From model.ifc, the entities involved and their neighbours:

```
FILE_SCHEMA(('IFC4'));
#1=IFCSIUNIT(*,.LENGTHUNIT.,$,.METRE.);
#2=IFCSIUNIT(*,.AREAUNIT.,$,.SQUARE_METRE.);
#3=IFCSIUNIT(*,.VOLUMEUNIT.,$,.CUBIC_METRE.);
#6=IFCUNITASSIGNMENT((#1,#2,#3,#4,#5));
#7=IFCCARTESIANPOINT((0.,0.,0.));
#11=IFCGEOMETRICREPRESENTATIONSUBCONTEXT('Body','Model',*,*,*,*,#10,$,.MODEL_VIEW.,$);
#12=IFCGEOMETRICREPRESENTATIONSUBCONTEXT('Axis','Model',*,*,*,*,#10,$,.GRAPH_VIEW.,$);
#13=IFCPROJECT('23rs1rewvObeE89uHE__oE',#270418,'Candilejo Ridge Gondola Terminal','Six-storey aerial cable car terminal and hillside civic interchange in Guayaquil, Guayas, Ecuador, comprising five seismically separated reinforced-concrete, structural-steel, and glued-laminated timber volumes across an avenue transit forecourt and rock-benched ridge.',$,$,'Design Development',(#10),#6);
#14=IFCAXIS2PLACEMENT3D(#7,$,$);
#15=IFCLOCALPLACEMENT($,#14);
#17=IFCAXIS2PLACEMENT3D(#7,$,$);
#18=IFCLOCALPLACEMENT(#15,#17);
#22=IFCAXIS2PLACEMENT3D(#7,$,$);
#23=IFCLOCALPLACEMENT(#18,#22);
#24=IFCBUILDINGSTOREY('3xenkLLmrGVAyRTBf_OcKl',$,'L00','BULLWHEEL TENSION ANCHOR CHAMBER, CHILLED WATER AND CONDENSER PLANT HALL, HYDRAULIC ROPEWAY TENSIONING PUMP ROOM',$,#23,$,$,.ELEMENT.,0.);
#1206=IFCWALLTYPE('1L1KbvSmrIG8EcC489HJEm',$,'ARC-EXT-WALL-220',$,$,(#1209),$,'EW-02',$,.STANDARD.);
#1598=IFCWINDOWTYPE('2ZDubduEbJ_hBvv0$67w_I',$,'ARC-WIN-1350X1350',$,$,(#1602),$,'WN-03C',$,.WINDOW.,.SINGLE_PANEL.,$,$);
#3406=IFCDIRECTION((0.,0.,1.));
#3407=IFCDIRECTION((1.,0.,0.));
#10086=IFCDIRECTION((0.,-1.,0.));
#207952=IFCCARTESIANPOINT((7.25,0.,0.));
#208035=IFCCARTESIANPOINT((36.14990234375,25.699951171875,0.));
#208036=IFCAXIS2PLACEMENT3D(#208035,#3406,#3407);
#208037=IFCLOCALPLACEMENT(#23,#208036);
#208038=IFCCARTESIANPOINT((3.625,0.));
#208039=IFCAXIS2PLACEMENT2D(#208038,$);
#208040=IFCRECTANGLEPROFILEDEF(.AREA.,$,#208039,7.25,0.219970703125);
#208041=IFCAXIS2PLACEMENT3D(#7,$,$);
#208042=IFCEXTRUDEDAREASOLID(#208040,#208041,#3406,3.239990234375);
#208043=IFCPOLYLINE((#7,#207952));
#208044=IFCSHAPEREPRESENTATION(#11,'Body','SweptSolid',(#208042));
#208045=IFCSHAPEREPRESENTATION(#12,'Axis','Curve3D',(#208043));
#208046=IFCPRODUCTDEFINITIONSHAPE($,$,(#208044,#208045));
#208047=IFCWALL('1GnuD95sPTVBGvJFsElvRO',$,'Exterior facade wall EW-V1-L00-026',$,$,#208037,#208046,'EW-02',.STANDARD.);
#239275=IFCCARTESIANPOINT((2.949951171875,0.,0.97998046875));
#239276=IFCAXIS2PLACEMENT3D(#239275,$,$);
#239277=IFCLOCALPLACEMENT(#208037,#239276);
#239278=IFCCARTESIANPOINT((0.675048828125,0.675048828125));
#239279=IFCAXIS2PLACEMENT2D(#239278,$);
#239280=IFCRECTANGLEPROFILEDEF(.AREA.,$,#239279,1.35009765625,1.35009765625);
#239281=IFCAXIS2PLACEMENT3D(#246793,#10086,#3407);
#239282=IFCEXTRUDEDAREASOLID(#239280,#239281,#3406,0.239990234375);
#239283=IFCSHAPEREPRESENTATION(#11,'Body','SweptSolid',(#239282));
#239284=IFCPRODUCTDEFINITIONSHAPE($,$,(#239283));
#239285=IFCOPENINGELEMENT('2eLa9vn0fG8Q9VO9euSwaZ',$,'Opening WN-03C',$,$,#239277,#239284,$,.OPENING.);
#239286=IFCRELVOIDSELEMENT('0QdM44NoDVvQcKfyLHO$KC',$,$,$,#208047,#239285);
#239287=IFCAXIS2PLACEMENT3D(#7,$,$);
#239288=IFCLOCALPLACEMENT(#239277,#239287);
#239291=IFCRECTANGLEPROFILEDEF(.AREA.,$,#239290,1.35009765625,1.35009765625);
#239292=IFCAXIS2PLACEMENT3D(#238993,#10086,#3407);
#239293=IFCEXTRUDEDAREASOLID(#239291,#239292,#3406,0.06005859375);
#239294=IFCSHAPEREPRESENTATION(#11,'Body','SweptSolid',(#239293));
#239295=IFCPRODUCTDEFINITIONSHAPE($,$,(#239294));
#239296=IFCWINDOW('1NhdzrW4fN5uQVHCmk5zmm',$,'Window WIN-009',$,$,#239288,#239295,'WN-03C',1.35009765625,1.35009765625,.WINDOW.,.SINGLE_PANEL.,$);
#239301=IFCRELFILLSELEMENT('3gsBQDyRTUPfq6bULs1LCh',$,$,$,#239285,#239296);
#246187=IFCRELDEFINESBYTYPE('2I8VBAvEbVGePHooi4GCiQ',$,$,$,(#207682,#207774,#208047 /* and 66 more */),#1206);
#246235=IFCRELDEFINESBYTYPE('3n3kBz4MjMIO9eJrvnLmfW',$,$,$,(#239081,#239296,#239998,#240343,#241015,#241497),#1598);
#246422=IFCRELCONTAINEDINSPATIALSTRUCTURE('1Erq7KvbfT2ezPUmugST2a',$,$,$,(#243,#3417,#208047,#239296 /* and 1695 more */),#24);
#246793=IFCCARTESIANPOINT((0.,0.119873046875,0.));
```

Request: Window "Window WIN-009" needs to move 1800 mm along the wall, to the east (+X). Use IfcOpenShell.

```python
import ifcopenshell
import ifcopenshell.api.geometry
import ifcopenshell.util.placement

model = ifcopenshell.open("model.ifc")

window = model.by_id(239296)
opening = window.FillsVoids[0].RelatingOpeningElement
wall = opening.VoidsElements[0].RelatingBuildingElement

wall_matrix = ifcopenshell.util.placement.get_local_placement(wall.ObjectPlacement)
shift = wall_matrix[:3, 0] * 1.8
before = ifcopenshell.util.placement.get_local_placement(window.ObjectPlacement)[:3, 3].copy()

# The window is placed relative to its opening, so it follows when the opening moves.
matrix = ifcopenshell.util.placement.get_local_placement(opening.ObjectPlacement)
matrix[:3, 3] += shift
ifcopenshell.api.geometry.edit_object_placement(
    model, product=opening, matrix=matrix, is_si=False, should_transform_children=True
)

after = ifcopenshell.util.placement.get_local_placement(window.ObjectPlacement)[:3, 3]
print("window moved by", (after - before).round(3) + 0.0)

model.write("model_rev.ifc")
```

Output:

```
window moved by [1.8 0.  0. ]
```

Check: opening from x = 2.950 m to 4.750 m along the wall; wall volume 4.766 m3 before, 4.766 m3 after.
